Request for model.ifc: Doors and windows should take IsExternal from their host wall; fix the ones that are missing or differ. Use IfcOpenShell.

First a look at what the model holds.

```python
import ifcopenshell
import ifcopenshell.util.element

model = ifcopenshell.open("model.ifc")
print(model.schema)
seen = {}
for e in model.by_type("IfcDoor") + model.by_type("IfcWindow"):
    if not e.FillsVoids:
        continue
    host = e.FillsVoids[0].RelatingOpeningElement.VoidsElements[0].RelatingBuildingElement
    own = ifcopenshell.util.element.get_pset(e, f"Pset_{e.is_a()[3:].removesuffix('StandardCase')}Common", "IsExternal")
    wall = ifcopenshell.util.element.get_pset(host, "Pset_WallCommon", "IsExternal")
    seen[e.is_a(), own, wall] = seen.get((e.is_a(), own, wall), 0) + 1
for (cls, own, wall), count in sorted(seen.items(), key=str):
    print(count, cls, "IsExternal:", own, "| host wall:", wall)
```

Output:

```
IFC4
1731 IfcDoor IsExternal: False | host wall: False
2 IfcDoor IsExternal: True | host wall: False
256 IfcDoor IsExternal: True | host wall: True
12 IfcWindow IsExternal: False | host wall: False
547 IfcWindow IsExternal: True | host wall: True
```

```python
import ifcopenshell
import ifcopenshell.api.pset
import ifcopenshell.util.element

model = ifcopenshell.open("model.ifc")

count = 0
for ifc_class, pset_name in (("IfcDoor", "Pset_DoorCommon"), ("IfcWindow", "Pset_WindowCommon")):
    for e in model.by_type(ifc_class):
        if not e.FillsVoids:
            continue
        host = e.FillsVoids[0].RelatingOpeningElement.VoidsElements[0].RelatingBuildingElement
        external = ifcopenshell.util.element.get_pset(host, "Pset_WallCommon", "IsExternal")
        if external is None or ifcopenshell.util.element.get_pset(e, pset_name, "IsExternal") == external:
            continue
        found = ifcopenshell.util.element.get_pset(e, pset_name, should_inherit=False)
        if found:
            pset = model.by_id(found["id"])
            if len(ifcopenshell.util.element.get_elements_by_pset(pset)) > 1:
                pset = ifcopenshell.api.pset.unshare_pset(model, products=[e], pset=pset)[0]
        else:
            pset = ifcopenshell.api.pset.add_pset(model, product=e, name=pset_name)
        ifcopenshell.api.pset.edit_pset(model, pset=pset, properties={"IsExternal": external})
        count += 1

print(count, "updated")

model.write("model_updated.ifc")
```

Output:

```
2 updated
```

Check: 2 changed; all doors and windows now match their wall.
